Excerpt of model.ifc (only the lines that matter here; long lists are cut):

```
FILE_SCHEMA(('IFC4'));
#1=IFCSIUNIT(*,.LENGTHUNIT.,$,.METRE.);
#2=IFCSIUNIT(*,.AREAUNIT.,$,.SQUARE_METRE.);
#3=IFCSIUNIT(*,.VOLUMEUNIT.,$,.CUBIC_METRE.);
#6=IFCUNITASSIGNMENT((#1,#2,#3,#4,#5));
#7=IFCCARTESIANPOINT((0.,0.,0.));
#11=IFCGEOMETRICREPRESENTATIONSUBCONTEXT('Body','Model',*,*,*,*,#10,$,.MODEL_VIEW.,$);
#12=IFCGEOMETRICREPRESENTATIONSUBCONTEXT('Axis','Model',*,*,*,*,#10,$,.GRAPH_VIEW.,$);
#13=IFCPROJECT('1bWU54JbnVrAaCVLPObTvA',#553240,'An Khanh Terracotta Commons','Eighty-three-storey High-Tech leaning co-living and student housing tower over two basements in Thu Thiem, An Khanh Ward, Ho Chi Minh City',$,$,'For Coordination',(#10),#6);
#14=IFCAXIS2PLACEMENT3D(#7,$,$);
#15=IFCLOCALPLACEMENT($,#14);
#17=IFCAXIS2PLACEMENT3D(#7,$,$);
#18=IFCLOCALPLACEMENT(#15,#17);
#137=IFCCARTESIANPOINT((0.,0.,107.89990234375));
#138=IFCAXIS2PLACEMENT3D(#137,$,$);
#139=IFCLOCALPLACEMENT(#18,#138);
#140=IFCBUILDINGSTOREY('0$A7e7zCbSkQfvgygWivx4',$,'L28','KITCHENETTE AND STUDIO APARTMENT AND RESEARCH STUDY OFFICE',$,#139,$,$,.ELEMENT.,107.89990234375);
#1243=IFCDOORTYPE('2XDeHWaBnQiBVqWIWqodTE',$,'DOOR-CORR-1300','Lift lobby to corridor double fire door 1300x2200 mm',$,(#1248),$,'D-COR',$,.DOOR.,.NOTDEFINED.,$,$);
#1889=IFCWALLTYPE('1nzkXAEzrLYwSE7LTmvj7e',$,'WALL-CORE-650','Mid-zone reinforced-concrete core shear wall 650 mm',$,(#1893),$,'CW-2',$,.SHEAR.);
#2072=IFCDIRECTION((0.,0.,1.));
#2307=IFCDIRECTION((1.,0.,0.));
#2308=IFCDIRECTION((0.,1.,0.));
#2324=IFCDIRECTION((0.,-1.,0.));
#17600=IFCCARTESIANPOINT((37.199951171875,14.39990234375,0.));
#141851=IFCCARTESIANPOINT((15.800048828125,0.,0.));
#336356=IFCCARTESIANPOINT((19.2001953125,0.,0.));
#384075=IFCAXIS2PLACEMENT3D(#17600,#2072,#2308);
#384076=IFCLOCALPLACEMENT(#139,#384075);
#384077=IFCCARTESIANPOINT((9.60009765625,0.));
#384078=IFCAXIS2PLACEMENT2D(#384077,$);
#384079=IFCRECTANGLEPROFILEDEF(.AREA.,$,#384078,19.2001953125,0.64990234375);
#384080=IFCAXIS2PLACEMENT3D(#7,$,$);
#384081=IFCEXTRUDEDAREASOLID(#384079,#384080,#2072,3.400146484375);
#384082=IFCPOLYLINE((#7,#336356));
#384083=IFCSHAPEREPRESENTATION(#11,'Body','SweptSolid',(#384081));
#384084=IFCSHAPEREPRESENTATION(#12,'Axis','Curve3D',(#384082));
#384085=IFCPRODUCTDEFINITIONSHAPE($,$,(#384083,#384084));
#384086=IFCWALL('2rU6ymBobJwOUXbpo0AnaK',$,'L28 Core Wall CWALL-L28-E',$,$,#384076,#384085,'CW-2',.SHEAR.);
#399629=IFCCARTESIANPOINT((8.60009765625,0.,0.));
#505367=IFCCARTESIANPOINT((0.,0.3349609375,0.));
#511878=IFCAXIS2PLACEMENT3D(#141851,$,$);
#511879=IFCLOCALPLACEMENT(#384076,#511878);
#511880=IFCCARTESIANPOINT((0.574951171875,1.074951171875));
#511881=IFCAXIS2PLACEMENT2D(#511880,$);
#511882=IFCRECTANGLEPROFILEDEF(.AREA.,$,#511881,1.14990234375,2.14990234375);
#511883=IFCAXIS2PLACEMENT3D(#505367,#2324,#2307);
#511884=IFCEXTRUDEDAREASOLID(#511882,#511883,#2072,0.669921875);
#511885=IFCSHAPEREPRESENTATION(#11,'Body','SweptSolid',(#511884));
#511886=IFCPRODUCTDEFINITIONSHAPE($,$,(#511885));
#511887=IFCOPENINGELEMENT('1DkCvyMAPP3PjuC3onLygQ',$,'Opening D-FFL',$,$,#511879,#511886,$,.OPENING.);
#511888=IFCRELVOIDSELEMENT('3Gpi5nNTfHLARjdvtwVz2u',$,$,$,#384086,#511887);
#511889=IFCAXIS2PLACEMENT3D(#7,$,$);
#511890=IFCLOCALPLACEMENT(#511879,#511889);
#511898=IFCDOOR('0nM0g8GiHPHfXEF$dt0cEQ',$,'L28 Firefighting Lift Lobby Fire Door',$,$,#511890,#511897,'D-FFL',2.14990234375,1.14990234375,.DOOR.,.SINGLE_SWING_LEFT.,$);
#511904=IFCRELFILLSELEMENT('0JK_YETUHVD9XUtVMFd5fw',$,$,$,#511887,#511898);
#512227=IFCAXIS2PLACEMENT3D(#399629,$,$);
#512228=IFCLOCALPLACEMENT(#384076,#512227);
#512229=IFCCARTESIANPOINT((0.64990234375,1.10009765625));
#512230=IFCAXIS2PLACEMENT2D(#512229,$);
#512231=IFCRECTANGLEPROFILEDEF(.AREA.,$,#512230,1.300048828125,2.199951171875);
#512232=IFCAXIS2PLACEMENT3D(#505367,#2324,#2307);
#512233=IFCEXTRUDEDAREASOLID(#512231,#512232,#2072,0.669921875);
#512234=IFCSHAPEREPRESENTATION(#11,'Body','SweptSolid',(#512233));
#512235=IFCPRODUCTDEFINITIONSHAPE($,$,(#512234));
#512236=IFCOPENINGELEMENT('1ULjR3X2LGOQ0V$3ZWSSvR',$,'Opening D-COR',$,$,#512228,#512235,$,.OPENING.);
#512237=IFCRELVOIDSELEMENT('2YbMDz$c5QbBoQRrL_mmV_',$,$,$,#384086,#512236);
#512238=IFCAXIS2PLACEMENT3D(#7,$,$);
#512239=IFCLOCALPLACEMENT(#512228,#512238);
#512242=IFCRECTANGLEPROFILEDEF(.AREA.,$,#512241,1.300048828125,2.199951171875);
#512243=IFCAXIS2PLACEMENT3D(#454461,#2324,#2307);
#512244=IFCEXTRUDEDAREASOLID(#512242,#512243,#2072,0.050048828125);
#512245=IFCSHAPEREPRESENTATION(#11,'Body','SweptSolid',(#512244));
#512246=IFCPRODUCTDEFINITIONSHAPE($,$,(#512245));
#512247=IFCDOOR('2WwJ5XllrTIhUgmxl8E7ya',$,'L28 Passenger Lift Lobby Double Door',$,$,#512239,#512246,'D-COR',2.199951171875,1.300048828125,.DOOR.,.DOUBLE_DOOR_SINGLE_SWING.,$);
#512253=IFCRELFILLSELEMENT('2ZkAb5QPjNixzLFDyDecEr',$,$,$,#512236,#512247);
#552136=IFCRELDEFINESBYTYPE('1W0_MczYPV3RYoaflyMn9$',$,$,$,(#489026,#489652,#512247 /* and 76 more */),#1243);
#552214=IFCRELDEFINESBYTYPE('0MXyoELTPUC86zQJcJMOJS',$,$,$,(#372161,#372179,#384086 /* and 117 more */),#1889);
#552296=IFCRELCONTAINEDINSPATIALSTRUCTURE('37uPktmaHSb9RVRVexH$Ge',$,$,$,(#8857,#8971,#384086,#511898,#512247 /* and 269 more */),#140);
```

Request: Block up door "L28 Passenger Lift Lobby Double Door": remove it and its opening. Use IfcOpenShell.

```python
import ifcopenshell
import ifcopenshell.api.feature
import ifcopenshell.api.root
import ifcopenshell.geom
import ifcopenshell.util.shape

model = ifcopenshell.open("model.ifc")
settings = ifcopenshell.geom.settings()


def volume(element):
    """Net volume in cubic metres, openings subtracted."""
    shape = ifcopenshell.geom.create_shape(settings, element)
    return ifcopenshell.util.shape.get_volume(shape.geometry)


door = model.by_id(512247)
opening = door.FillsVoids[0].RelatingOpeningElement
wall = opening.VoidsElements[0].RelatingBuildingElement
before = volume(wall)

ifcopenshell.api.root.remove_product(model, product=door)
ifcopenshell.api.feature.remove_feature(model, feature=opening)

after = volume(wall)

print(f"wall volume {before:.3f} -> {after:.3f} m3")

model.write("model_edited.ifc")
```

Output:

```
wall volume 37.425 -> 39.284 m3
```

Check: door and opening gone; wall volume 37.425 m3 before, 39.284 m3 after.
